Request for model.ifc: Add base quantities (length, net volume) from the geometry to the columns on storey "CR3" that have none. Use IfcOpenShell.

First a look at what the model holds.

```python
import ifcopenshell
import ifcopenshell.util.element
import ifcopenshell.util.unit

model = ifcopenshell.open("model.ifc")
print(model.schema)
for unit_type in ("LENGTHUNIT", "AREAUNIT", "VOLUMEUNIT"):
    print(unit_type, ifcopenshell.util.unit.calculate_unit_scale(model, unit_type))
storey = next(s for s in model.by_type("IfcBuildingStorey") if s.Name == "CR3")
columns = [e for e in ifcopenshell.util.element.get_decomposition(storey) if e.is_a("IfcColumn")]
for e in sorted(columns, key=lambda e: e.id()):
    print(e.id(), e.is_a(), e.Name, list(ifcopenshell.util.element.get_psets(e, qtos_only=True)), sep=" | ")
```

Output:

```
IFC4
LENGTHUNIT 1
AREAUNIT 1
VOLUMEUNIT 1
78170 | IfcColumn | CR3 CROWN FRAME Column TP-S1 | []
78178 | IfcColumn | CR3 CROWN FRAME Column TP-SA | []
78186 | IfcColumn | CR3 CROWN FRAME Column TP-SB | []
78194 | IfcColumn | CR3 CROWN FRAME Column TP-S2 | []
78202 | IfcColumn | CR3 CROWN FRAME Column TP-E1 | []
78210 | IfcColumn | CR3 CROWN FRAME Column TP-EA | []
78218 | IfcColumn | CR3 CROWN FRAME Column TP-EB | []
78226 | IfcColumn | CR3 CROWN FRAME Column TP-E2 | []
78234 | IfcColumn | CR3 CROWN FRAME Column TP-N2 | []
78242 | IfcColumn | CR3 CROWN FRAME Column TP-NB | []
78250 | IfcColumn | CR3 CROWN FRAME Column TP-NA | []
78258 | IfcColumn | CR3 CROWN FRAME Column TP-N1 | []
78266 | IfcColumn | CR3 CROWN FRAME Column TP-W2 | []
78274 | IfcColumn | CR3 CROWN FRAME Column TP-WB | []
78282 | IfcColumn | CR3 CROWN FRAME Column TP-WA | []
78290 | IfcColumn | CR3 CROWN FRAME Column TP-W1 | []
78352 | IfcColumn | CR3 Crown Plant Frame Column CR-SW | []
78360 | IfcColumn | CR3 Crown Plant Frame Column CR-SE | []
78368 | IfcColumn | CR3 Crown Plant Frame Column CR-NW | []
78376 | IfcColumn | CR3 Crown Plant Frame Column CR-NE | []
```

```python
import ifcopenshell
import ifcopenshell.api.pset
import ifcopenshell.geom
import ifcopenshell.util.element
import ifcopenshell.util.shape
import ifcopenshell.util.unit

model = ifcopenshell.open("model.ifc")
unit_scale = ifcopenshell.util.unit.calculate_unit_scale(model)
volume_scale = ifcopenshell.util.unit.calculate_unit_scale(model, "VOLUMEUNIT")
settings = ifcopenshell.geom.settings()

storey = next(s for s in model.by_type("IfcBuildingStorey") if s.Name == "CR3")
columns = [e for e in ifcopenshell.util.element.get_decomposition(storey) if e.is_a("IfcColumn")]

for e in sorted(columns, key=lambda e: e.id()):
    if ifcopenshell.util.element.get_psets(e, qtos_only=True, should_inherit=False):
        continue
    # Geometry comes back in metres, in the element's own axes.
    shape = ifcopenshell.geom.create_shape(settings, e)
    values = {
        "Length": ifcopenshell.util.shape.get_z(shape.geometry) / unit_scale,
        "NetVolume": ifcopenshell.util.shape.get_volume(shape.geometry) / volume_scale,
    }
    qto = ifcopenshell.api.pset.add_qto(model, product=e, name="Qto_ColumnBaseQuantities")
    ifcopenshell.api.pset.edit_qto(model, qto=qto, properties=values)
    print(e.id(), {k: round(v, 3) for k, v in values.items()})

model.write("model_rev.ifc")
```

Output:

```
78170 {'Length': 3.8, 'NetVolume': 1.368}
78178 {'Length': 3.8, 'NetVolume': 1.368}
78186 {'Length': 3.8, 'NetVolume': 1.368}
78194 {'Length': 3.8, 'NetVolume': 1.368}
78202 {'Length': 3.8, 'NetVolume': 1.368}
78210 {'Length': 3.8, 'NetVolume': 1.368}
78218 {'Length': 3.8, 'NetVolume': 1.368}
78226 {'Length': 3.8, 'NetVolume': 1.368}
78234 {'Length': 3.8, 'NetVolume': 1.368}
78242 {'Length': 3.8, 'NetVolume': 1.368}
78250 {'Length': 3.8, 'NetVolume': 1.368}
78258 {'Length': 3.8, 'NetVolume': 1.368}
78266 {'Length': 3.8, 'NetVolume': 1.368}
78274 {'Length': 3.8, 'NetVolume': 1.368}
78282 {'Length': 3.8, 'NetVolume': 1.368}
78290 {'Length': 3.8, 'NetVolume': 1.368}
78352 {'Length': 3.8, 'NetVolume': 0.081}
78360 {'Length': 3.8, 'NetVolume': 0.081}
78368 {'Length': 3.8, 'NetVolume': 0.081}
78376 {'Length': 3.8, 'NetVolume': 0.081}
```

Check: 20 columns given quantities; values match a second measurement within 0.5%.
